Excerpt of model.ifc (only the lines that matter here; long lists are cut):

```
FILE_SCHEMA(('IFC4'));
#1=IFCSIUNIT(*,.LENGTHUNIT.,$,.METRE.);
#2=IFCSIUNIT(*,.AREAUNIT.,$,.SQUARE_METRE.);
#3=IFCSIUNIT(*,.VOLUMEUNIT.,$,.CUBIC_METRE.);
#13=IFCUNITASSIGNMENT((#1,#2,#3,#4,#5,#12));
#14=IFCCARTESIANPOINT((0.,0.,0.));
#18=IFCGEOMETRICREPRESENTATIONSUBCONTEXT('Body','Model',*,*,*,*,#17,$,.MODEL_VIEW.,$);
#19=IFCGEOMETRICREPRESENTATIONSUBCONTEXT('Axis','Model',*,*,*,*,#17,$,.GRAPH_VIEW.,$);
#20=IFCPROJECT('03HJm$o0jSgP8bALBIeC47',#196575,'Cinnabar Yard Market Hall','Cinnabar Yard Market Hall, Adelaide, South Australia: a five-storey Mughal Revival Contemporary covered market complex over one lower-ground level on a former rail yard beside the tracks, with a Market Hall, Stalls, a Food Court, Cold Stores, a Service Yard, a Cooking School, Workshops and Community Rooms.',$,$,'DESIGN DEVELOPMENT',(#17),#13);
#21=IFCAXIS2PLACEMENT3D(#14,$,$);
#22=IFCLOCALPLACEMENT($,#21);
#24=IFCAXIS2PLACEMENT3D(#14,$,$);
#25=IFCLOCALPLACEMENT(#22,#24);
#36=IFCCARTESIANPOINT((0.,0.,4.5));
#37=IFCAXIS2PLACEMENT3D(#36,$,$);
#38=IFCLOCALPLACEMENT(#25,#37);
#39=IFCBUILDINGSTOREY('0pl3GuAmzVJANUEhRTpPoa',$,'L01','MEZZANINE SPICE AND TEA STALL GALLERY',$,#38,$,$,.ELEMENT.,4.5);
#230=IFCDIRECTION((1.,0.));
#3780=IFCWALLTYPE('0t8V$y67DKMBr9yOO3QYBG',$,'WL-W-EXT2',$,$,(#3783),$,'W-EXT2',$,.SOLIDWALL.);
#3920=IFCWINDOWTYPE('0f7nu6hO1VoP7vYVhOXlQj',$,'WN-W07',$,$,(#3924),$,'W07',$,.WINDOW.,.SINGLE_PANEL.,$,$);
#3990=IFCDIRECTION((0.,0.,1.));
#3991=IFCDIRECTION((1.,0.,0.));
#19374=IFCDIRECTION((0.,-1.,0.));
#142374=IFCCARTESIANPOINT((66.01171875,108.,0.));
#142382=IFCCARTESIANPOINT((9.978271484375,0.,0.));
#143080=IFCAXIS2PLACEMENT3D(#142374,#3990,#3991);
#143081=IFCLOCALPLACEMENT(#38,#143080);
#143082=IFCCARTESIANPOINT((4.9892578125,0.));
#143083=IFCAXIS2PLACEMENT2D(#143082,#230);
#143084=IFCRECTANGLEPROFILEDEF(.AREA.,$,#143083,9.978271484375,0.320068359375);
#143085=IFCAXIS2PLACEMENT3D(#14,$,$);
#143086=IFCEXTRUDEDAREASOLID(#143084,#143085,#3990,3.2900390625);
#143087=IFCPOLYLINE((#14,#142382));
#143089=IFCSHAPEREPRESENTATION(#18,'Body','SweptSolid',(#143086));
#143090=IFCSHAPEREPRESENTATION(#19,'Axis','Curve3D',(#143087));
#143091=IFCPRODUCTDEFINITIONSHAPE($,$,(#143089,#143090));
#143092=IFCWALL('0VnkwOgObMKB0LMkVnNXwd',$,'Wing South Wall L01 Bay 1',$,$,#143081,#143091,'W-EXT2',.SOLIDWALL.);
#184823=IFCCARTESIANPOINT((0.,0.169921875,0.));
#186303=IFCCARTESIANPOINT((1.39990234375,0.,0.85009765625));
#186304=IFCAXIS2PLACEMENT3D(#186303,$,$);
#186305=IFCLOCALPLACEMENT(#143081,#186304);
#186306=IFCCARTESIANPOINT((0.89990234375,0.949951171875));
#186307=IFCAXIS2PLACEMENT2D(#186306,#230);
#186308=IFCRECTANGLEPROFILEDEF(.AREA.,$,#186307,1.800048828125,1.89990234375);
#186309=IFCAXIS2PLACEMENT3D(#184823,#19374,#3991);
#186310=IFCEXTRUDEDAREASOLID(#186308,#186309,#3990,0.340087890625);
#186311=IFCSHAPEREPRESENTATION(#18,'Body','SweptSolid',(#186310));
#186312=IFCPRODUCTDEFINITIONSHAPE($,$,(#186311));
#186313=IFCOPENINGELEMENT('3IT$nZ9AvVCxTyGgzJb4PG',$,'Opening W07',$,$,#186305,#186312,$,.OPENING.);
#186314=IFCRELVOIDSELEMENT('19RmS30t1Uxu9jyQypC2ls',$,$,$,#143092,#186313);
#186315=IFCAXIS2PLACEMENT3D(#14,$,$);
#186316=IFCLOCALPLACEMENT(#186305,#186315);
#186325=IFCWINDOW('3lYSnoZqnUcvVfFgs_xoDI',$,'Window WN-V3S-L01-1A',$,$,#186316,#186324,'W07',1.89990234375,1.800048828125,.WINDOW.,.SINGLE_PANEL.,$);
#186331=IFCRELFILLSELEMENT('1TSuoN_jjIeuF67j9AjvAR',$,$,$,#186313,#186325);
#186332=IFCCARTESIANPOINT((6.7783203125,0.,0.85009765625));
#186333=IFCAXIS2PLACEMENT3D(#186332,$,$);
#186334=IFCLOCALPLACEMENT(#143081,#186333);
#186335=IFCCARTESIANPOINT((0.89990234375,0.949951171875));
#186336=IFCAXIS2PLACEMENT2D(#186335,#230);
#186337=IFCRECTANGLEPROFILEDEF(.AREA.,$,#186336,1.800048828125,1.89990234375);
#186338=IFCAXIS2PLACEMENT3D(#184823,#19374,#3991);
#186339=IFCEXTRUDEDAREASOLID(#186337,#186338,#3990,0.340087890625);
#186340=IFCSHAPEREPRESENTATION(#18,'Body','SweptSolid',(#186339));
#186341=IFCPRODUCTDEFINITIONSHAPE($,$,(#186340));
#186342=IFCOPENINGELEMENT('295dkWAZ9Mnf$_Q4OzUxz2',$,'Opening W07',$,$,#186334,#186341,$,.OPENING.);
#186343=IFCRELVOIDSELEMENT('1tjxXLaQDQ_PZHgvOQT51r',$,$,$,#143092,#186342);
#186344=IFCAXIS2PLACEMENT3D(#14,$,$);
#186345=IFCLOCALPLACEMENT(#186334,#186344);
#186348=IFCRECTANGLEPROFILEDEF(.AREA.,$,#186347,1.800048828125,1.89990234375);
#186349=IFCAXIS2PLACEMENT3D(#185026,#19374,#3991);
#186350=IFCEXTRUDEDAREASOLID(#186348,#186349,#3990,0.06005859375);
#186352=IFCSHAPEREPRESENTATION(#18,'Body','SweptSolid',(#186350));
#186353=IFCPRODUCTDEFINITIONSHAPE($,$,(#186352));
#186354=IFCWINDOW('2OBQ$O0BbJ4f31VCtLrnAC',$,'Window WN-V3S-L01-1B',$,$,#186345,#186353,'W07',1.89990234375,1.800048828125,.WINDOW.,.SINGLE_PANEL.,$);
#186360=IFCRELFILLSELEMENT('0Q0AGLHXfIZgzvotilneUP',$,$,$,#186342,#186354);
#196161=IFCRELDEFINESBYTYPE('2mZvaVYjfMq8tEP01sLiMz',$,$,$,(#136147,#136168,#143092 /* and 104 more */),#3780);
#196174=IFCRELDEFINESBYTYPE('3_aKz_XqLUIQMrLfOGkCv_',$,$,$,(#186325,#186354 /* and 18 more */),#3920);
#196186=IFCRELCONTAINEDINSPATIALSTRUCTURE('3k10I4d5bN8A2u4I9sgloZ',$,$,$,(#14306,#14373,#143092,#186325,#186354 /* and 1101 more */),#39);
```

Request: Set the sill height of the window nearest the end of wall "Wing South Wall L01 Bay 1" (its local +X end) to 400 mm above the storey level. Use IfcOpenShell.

```python
import numpy as np
import ifcopenshell
import ifcopenshell.api.geometry
import ifcopenshell.geom
import ifcopenshell.util.element
import ifcopenshell.util.placement
import ifcopenshell.util.shape
import ifcopenshell.util.unit

model = ifcopenshell.open("model.ifc")
unit_scale = ifcopenshell.util.unit.calculate_unit_scale(model)

window = model.by_id(186354)
opening = window.FillsVoids[0].RelatingOpeningElement
storey = ifcopenshell.util.element.get_container(window, ifc_class="IfcBuildingStorey")
level = ifcopenshell.util.placement.get_local_placement(storey.ObjectPlacement)[2, 3]

# The opening's origin need not be at the sill, so measure its lowest point.
shape = ifcopenshell.geom.create_shape(ifcopenshell.geom.settings(), opening)
bottom = ifcopenshell.util.shape.get_shape_bottom_elevation(shape, shape.geometry) / unit_scale
dz = level + 0.4 / unit_scale - bottom

shift = np.array([0.0, 0.0, dz])
# The window is placed relative to its opening, so it follows when the opening moves.
matrix = ifcopenshell.util.placement.get_local_placement(opening.ObjectPlacement)
matrix[:3, 3] += shift
ifcopenshell.api.geometry.edit_object_placement(
    model, product=opening, matrix=matrix, is_si=False, should_transform_children=True
)

print(f"moved by {dz * unit_scale:+.3f} m")

model.write("model_rev.ifc")
```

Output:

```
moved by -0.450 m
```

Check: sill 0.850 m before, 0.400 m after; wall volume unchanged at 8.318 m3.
